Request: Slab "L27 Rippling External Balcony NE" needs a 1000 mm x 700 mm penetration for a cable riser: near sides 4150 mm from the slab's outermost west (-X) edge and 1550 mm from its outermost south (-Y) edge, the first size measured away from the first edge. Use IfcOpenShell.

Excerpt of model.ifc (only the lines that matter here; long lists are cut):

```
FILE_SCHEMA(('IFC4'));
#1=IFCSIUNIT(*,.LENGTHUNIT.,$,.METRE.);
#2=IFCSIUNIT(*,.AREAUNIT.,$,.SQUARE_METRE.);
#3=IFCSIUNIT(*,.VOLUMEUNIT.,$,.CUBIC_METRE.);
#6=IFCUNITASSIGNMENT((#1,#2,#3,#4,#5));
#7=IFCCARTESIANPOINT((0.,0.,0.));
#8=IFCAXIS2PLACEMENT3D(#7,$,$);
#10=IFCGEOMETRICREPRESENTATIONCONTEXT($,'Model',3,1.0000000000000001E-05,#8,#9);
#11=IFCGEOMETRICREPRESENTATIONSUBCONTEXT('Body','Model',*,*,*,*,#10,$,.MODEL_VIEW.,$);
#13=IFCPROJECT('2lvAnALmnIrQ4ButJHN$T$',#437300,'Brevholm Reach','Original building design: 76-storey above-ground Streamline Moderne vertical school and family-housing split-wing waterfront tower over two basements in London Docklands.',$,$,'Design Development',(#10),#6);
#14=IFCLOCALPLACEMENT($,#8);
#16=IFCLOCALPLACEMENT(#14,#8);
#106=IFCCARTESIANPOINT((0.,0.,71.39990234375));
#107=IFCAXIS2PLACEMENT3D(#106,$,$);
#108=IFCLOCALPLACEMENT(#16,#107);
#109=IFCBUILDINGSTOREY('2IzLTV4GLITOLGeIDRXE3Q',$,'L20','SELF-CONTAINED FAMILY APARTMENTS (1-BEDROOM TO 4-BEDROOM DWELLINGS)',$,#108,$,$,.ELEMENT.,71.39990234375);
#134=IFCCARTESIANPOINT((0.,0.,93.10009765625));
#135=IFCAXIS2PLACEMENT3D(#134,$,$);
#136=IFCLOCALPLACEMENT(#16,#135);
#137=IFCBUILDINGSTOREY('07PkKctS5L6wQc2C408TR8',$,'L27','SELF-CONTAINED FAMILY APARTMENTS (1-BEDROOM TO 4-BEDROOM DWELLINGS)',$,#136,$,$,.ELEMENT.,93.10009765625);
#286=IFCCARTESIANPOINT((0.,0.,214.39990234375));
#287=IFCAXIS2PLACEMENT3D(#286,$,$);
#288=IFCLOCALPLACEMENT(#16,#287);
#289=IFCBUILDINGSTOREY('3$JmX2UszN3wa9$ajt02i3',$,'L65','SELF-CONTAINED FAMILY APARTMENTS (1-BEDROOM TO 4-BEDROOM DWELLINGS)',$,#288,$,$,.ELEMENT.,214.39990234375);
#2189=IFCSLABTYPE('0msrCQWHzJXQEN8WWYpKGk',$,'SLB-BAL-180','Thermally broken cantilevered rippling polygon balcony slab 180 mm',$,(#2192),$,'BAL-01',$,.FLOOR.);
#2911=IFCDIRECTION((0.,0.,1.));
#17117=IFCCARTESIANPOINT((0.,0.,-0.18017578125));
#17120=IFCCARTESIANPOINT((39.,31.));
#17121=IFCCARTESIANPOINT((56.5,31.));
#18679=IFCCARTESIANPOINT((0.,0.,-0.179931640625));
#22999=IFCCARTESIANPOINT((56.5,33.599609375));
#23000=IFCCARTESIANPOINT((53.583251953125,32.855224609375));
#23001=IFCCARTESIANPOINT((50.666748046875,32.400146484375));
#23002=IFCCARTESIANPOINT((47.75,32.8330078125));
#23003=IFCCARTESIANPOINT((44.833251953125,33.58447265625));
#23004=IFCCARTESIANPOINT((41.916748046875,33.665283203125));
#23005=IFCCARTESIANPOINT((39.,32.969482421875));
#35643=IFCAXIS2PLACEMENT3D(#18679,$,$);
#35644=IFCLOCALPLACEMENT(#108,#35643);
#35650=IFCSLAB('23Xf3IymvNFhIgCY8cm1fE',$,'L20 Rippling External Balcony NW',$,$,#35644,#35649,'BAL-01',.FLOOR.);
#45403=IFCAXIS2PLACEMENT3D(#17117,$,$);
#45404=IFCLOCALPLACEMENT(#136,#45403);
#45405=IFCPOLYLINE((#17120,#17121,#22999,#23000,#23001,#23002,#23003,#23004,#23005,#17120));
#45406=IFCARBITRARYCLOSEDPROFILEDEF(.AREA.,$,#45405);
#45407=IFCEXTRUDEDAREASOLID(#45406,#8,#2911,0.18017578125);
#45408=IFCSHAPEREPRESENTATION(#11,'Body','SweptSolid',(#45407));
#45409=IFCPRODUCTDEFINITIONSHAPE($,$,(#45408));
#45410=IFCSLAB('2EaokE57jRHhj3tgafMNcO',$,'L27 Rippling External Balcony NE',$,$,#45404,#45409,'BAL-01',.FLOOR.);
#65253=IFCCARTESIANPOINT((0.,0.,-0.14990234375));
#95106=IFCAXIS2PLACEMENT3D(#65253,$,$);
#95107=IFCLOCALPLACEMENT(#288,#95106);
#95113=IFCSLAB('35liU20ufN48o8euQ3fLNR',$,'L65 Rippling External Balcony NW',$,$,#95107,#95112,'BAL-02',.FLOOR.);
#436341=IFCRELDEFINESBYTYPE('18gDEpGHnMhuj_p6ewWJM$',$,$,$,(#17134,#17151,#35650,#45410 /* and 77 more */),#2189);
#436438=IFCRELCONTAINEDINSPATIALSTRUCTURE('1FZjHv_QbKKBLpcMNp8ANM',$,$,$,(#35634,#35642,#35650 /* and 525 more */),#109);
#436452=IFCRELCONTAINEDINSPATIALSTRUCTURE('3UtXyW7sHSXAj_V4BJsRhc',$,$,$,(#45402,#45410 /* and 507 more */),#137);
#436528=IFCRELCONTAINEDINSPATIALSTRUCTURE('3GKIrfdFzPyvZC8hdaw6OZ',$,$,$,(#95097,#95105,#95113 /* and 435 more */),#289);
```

```python
import numpy as np
import ifcopenshell
import ifcopenshell.api.feature
import ifcopenshell.api.geometry
import ifcopenshell.api.root
import ifcopenshell.geom
import ifcopenshell.util.placement
import ifcopenshell.util.representation
import ifcopenshell.util.shape
import ifcopenshell.util.unit

model = ifcopenshell.open("model.ifc")
unit_scale = ifcopenshell.util.unit.calculate_unit_scale(model)
settings = ifcopenshell.geom.settings()


def volume(element):
    """Net volume in cubic metres, openings subtracted."""
    shape = ifcopenshell.geom.create_shape(settings, element)
    return ifcopenshell.util.shape.get_volume(shape.geometry)


slab = model.by_guid("2EaokE57jRHhj3tgafMNcO")
before = volume(slab)

# Extent in the slab's own axes, in metres. The edges named are its -X and -Y sides.
slab_shape = ifcopenshell.geom.create_shape(settings, slab)
vertices = ifcopenshell.util.shape.get_vertices(slab_shape.geometry)
x_min, y_min, bottom = vertices.min(axis=0)
top = vertices[:, 2].max()

opening = ifcopenshell.api.root.create_entity(model, ifc_class="IfcOpeningElement", name="Cable riser opening", predefined_type="OPENING")
context = ifcopenshell.util.representation.get_context(model, "Model", "Body", "MODEL_VIEW")
width, depth = 1, 0.7
outline = [(0.0, 0.0), (width, 0.0), (width, depth), (0.0, depth), (0.0, 0.0)]
# Overshoot both faces by 50 mm so the cut is clean.
shape = ifcopenshell.api.geometry.add_slab_representation(
    model, context=context, depth=top - bottom + 0.1, polyline=outline
)
ifcopenshell.api.geometry.assign_representation(model, product=opening, representation=shape)

matrix = ifcopenshell.util.placement.get_local_placement(slab.ObjectPlacement)
matrix[:, 3] = matrix @ np.append(np.array([x_min + 4.15, y_min + 1.55, bottom - 0.05]) / unit_scale, 1.0)
ifcopenshell.api.geometry.edit_object_placement(model, product=opening, matrix=matrix, is_si=False)
ifcopenshell.api.feature.add_feature(model, feature=opening, element=slab)

after = volume(slab)

print(f"slab volume {before:.3f} -> {after:.3f} m3")

model.write("model_v2.ifc")
```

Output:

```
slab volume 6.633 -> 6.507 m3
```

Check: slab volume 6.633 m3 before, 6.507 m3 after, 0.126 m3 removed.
